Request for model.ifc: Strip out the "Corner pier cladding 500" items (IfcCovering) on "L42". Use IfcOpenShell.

First a look at what the model holds.

```python
import ifcopenshell
import ifcopenshell.util.element

model = ifcopenshell.open("model.ifc")
print(model.schema)
storey = next(s for s in model.by_type("IfcBuildingStorey") if s.Name == "L42")
coverings = [e for e in ifcopenshell.util.element.get_decomposition(storey) if e.is_a("IfcCovering")]
seen = {}
for e in coverings:
    element_type = ifcopenshell.util.element.get_type(e)
    name = element_type.Name if element_type not in (None, e) else None
    seen[name] = seen.get(name, 0) + 1
for name, count in sorted(seen.items(), key=str):
    print(count, "x", name)
```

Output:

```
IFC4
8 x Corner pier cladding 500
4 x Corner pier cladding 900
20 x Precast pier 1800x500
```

```python
import ifcopenshell
import ifcopenshell.api.root
import ifcopenshell.util.element

model = ifcopenshell.open("model.ifc")

storey = next(s for s in model.by_type("IfcBuildingStorey") if s.Name == "L42")
coverings = [e for e in ifcopenshell.util.element.get_decomposition(storey) if e.is_a("IfcCovering")]
targets = [e for e in coverings if (t := ifcopenshell.util.element.get_type(e)) not in (None, e) and t.Name == "Corner pier cladding 500"]

for e in targets:
    ifcopenshell.api.root.remove_product(model, product=e)
print(len(targets), "removed")

model.write("model_v2.ifc")
```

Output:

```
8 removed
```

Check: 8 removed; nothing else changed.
